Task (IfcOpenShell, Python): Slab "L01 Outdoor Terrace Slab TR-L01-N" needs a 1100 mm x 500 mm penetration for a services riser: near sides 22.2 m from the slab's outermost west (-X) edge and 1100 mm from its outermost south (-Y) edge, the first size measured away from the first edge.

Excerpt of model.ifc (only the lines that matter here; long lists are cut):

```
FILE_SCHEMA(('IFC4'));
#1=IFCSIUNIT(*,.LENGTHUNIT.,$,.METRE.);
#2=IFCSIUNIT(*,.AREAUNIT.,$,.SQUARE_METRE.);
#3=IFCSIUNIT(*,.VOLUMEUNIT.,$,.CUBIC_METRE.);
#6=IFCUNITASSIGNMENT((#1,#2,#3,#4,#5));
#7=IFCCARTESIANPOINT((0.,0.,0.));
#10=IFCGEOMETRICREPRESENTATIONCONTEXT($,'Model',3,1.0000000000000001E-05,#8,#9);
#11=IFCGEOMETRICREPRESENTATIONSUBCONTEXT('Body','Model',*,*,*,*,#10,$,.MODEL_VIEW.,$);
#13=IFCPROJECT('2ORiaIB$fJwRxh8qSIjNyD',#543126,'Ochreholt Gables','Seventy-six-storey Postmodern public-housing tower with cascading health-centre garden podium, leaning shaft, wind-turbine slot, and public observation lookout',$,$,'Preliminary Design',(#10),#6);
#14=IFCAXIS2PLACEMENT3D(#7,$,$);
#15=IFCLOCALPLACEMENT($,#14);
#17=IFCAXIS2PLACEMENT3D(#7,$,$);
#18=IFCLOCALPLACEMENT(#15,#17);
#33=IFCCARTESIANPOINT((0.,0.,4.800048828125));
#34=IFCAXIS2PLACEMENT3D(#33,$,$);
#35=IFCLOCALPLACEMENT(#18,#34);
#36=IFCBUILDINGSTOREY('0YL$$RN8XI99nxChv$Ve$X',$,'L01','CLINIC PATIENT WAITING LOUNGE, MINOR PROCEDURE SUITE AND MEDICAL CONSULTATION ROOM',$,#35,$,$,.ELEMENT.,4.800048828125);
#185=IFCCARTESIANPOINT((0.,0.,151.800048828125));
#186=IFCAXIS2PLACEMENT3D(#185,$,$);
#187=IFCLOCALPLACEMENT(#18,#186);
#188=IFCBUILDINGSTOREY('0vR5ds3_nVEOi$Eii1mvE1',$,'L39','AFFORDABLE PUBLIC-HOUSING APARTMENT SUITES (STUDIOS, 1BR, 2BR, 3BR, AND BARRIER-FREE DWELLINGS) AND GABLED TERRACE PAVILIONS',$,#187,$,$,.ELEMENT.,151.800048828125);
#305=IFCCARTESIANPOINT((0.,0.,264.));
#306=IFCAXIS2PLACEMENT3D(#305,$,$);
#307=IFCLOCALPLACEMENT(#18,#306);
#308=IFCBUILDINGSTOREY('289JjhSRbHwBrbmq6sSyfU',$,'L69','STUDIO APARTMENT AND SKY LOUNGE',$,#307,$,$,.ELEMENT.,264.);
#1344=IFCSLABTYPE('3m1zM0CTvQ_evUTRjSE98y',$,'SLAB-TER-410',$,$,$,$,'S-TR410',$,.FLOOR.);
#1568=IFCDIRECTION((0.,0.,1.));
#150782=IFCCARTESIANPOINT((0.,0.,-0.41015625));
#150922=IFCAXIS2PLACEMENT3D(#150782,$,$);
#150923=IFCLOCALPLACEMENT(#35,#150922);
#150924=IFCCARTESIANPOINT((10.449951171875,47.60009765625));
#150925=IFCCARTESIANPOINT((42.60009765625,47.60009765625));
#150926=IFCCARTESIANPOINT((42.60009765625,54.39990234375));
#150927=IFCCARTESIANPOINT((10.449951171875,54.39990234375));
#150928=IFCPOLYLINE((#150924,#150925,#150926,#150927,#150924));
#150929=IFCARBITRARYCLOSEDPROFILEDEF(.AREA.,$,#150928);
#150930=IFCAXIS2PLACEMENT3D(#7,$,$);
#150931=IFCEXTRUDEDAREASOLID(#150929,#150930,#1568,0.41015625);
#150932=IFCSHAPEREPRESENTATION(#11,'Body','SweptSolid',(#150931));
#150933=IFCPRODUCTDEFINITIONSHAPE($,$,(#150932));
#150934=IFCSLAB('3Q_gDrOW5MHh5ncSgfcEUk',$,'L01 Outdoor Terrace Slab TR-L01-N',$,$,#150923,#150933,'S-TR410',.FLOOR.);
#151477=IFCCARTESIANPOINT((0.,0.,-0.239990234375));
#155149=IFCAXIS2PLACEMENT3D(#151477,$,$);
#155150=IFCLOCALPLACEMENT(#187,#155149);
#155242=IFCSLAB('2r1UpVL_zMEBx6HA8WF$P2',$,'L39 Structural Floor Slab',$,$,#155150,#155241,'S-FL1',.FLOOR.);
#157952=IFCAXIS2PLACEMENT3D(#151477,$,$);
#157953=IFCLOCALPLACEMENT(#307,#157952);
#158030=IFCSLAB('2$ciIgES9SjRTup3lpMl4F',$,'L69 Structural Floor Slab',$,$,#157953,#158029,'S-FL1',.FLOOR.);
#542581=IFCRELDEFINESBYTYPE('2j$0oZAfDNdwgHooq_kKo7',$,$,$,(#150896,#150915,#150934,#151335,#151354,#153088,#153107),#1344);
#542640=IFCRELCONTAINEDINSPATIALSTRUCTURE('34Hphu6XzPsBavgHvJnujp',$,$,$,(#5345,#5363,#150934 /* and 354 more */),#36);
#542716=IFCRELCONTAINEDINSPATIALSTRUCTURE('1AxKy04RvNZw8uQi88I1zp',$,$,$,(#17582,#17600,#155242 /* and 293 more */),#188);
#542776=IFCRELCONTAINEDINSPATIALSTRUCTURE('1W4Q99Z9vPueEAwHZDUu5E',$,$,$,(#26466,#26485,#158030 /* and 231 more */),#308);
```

```python
import numpy as np
import ifcopenshell
import ifcopenshell.api.feature
import ifcopenshell.api.geometry
import ifcopenshell.api.root
import ifcopenshell.geom
import ifcopenshell.util.placement
import ifcopenshell.util.representation
import ifcopenshell.util.shape
import ifcopenshell.util.unit

model = ifcopenshell.open("model.ifc")
unit_scale = ifcopenshell.util.unit.calculate_unit_scale(model)
settings = ifcopenshell.geom.settings()


def volume(element):
    """Net volume in cubic metres, openings subtracted."""
    shape = ifcopenshell.geom.create_shape(settings, element)
    return ifcopenshell.util.shape.get_volume(shape.geometry)


slab = model.by_guid("3Q_gDrOW5MHh5ncSgfcEUk")
before = volume(slab)

# Extent in the slab's own axes, in metres. The edges named are its -X and -Y sides.
slab_shape = ifcopenshell.geom.create_shape(settings, slab)
vertices = ifcopenshell.util.shape.get_vertices(slab_shape.geometry)
x_min, y_min, bottom = vertices.min(axis=0)
top = vertices[:, 2].max()

opening = ifcopenshell.api.root.create_entity(model, ifc_class="IfcOpeningElement", name="Services riser opening", predefined_type="OPENING")
context = ifcopenshell.util.representation.get_context(model, "Model", "Body", "MODEL_VIEW")
width, depth = 1.1, 0.5
outline = [(0.0, 0.0), (width, 0.0), (width, depth), (0.0, depth), (0.0, 0.0)]
# Overshoot both faces by 50 mm so the cut is clean.
shape = ifcopenshell.api.geometry.add_slab_representation(
    model, context=context, depth=top - bottom + 0.1, polyline=outline
)
ifcopenshell.api.geometry.assign_representation(model, product=opening, representation=shape)

matrix = ifcopenshell.util.placement.get_local_placement(slab.ObjectPlacement)
matrix[:, 3] = matrix @ np.append(np.array([x_min + 22.2, y_min + 1.1, bottom - 0.05]) / unit_scale, 1.0)
ifcopenshell.api.geometry.edit_object_placement(model, product=opening, matrix=matrix, is_si=False)
ifcopenshell.api.feature.add_feature(model, feature=opening, element=slab)

after = volume(slab)

print(f"slab volume {before:.3f} -> {after:.3f} m3")

model.write("model-out.ifc")
```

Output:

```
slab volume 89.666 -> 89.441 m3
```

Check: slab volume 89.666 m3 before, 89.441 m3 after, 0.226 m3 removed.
